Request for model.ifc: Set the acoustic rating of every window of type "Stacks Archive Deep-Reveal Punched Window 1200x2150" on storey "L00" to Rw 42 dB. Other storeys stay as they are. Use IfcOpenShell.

First a look at what the model holds.

```python
import ifcopenshell
import ifcopenshell.util.element

model = ifcopenshell.open("model.ifc")
print(model.schema)
storey = next(s for s in model.by_type("IfcBuildingStorey") if s.Name == "L00")
windows = [e for e in ifcopenshell.util.element.get_decomposition(storey) if e.is_a("IfcWindow")]
seen = {}
for e in windows:
    element_type = ifcopenshell.util.element.get_type(e)
    key = (element_type.Name if element_type != e and element_type else None, ifcopenshell.util.element.get_pset(e, "Pset_WindowCommon", "AcousticRating"))
    seen[key] = seen.get(key, 0) + 1
for (name, value), count in sorted(seen.items(), key=str):
    print(count, "x", name, "|", value)
```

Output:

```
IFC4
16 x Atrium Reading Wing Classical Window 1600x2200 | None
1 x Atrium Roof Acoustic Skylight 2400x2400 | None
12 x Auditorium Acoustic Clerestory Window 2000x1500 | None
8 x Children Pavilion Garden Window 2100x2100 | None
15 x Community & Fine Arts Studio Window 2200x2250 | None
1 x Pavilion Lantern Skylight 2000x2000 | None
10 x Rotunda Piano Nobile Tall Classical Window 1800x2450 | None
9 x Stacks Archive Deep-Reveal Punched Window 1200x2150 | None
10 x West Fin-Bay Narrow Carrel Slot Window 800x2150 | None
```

```python
import ifcopenshell
import ifcopenshell.api.pset
import ifcopenshell.util.element

model = ifcopenshell.open("model.ifc")

storey = next(s for s in model.by_type("IfcBuildingStorey") if s.Name == "L00")
windows = [e for e in ifcopenshell.util.element.get_decomposition(storey) if e.is_a("IfcWindow")]

count = 0
for e in windows:
    element_type = ifcopenshell.util.element.get_type(e)
    if element_type in (None, e) or element_type.Name != "Stacks Archive Deep-Reveal Punched Window 1200x2150":
        continue
    # add_pset returns the element's existing set when there is one.
    pset = ifcopenshell.api.pset.add_pset(model, product=e, name="Pset_WindowCommon")
    ifcopenshell.api.pset.edit_pset(model, pset=pset, properties={"AcousticRating": "Rw 42 dB"})
    count += 1

print(count, "windows updated")

model.write("model_edited.ifc")
```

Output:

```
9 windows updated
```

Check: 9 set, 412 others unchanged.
